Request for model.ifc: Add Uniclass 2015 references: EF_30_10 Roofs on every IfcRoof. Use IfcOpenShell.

First a look at what the model holds.

```python
import ifcopenshell

model = ifcopenshell.open("model.ifc")
print(model.schema)
print("classifications:", [c.Name for c in model.by_type("IfcClassification")])
for ifc_class in ("IfcDoor", "IfcRoof", "IfcStair", "IfcWall", "IfcWindow"):
    print(ifc_class, len(model.by_type(ifc_class)))
```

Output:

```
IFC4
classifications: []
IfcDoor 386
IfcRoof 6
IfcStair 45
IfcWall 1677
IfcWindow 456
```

```python
import ifcopenshell
import ifcopenshell.api.classification

model = ifcopenshell.open("model.ifc")

system = ifcopenshell.api.classification.add_classification(model, classification="Uniclass 2015")

codes = {
    "IfcRoof": ("EF_30_10", "Roofs"),
}
for ifc_class, (code, name) in codes.items():
    products = model.by_type(ifc_class)
    ifcopenshell.api.classification.add_reference(
        model, products=products, classification=system, identification=code, name=name
    )
    print(code, len(products))

model.write("model_rev.ifc")
```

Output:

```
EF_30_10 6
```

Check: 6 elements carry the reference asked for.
